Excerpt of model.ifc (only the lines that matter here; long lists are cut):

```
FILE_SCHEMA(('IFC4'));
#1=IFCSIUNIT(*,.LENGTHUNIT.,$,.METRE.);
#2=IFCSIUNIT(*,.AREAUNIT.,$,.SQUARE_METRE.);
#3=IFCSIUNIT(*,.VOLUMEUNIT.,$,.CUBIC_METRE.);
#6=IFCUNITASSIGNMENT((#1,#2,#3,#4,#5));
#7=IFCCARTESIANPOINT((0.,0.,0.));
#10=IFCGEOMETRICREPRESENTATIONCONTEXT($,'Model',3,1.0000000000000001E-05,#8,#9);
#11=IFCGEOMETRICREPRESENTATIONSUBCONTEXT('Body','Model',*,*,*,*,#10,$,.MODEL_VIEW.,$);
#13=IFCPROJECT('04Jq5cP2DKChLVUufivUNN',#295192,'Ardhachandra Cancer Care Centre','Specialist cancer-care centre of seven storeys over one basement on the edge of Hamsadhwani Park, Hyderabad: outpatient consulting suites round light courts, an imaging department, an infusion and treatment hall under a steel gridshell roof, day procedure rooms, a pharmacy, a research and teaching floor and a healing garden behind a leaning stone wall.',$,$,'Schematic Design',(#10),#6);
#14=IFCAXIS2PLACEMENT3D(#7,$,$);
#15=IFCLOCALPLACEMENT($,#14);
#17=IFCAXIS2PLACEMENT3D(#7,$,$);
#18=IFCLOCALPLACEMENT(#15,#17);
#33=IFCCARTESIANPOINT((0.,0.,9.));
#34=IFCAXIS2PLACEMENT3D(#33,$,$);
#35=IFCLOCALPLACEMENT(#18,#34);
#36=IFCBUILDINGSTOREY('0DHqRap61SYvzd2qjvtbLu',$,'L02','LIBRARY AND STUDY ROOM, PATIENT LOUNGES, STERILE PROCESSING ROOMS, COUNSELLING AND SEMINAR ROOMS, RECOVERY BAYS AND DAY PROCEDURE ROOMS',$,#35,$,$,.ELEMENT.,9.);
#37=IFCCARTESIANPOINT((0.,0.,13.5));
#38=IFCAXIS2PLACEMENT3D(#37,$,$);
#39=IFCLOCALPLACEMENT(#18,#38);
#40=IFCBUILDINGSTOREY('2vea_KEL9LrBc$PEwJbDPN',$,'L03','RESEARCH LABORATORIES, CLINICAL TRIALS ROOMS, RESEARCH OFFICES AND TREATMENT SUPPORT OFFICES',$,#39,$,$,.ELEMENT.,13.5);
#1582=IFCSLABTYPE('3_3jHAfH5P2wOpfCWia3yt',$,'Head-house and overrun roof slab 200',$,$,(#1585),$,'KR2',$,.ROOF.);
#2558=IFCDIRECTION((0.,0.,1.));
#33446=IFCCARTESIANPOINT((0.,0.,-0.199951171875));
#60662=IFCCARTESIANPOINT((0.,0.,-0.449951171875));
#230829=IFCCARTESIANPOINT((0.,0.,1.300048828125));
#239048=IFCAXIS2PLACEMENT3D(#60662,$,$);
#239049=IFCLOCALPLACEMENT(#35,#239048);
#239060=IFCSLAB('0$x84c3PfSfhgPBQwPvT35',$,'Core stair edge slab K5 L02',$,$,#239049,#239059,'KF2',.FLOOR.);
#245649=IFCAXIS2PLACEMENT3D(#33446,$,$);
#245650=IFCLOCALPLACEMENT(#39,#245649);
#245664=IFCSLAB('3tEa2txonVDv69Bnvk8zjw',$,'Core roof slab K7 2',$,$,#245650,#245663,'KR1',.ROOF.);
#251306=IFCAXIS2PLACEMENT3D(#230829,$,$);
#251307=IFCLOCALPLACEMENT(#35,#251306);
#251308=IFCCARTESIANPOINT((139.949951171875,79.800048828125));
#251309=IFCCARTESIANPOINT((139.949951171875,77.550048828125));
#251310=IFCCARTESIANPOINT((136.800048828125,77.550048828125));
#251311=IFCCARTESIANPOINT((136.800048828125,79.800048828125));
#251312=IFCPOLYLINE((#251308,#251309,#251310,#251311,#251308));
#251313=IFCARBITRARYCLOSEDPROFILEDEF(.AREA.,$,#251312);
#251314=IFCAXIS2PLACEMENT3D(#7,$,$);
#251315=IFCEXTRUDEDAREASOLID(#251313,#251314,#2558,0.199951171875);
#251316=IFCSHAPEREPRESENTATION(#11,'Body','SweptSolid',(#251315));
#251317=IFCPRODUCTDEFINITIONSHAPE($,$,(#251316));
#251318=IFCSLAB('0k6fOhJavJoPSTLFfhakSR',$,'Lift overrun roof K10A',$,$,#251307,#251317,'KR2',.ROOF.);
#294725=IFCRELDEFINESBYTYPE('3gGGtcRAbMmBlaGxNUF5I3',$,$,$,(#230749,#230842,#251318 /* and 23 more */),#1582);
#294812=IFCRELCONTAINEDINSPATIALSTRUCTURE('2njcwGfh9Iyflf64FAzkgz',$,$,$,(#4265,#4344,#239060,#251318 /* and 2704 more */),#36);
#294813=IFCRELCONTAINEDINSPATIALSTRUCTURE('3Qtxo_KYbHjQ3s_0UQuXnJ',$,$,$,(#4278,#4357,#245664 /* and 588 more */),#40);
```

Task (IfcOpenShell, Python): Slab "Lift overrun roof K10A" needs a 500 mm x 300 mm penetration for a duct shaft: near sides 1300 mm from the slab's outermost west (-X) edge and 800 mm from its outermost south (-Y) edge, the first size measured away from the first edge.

```python
import numpy as np
import ifcopenshell
import ifcopenshell.api.feature
import ifcopenshell.api.geometry
import ifcopenshell.api.root
import ifcopenshell.geom
import ifcopenshell.util.placement
import ifcopenshell.util.representation
import ifcopenshell.util.shape
import ifcopenshell.util.unit

model = ifcopenshell.open("model.ifc")
unit_scale = ifcopenshell.util.unit.calculate_unit_scale(model)
settings = ifcopenshell.geom.settings()


def volume(element):
    """Net volume in cubic metres, openings subtracted."""
    shape = ifcopenshell.geom.create_shape(settings, element)
    return ifcopenshell.util.shape.get_volume(shape.geometry)


slab = model.by_guid("0k6fOhJavJoPSTLFfhakSR")
before = volume(slab)

# Extent in the slab's own axes, in metres. The edges named are its -X and -Y sides.
slab_shape = ifcopenshell.geom.create_shape(settings, slab)
vertices = ifcopenshell.util.shape.get_vertices(slab_shape.geometry)
x_min, y_min, bottom = vertices.min(axis=0)
top = vertices[:, 2].max()

opening = ifcopenshell.api.root.create_entity(model, ifc_class="IfcOpeningElement", name="Duct shaft opening", predefined_type="OPENING")
context = ifcopenshell.util.representation.get_context(model, "Model", "Body", "MODEL_VIEW")
width, depth = 0.5, 0.3
outline = [(0.0, 0.0), (width, 0.0), (width, depth), (0.0, depth), (0.0, 0.0)]
# Overshoot both faces by 50 mm so the cut is clean.
shape = ifcopenshell.api.geometry.add_slab_representation(
    model, context=context, depth=top - bottom + 0.1, polyline=outline
)
ifcopenshell.api.geometry.assign_representation(model, product=opening, representation=shape)

matrix = ifcopenshell.util.placement.get_local_placement(slab.ObjectPlacement)
matrix[:, 3] = matrix @ np.append(np.array([x_min + 1.3, y_min + 0.8, bottom - 0.05]) / unit_scale, 1.0)
ifcopenshell.api.geometry.edit_object_placement(model, product=opening, matrix=matrix, is_si=False)
ifcopenshell.api.feature.add_feature(model, feature=opening, element=slab)

after = volume(slab)

print(f"slab volume {before:.3f} -> {after:.3f} m3")

model.write("model_updated.ifc")
```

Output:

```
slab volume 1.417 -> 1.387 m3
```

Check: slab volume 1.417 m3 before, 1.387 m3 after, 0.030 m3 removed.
